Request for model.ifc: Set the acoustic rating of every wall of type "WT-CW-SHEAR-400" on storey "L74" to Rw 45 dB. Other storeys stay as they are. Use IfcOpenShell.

First a look at what the model holds.

```python
import ifcopenshell
import ifcopenshell.util.element

model = ifcopenshell.open("model.ifc")
print(model.schema)
storey = next(s for s in model.by_type("IfcBuildingStorey") if s.Name == "L74")
walls = [e for e in ifcopenshell.util.element.get_decomposition(storey) if e.is_a("IfcWall")]
seen = {}
for e in walls:
    element_type = ifcopenshell.util.element.get_type(e)
    key = (element_type.Name if element_type != e and element_type else None, ifcopenshell.util.element.get_pset(e, "Pset_WallCommon", "AcousticRating"))
    seen[key] = seen.get(key, 0) + 1
for (name, value), count in sorted(seen.items(), key=str):
    print(count, "x", name, "|", value)
```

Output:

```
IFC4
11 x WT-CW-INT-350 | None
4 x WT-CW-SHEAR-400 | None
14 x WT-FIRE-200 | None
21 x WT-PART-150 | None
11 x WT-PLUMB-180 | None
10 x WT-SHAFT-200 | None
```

```python
import ifcopenshell
import ifcopenshell.api.pset
import ifcopenshell.util.element

model = ifcopenshell.open("model.ifc")

storey = next(s for s in model.by_type("IfcBuildingStorey") if s.Name == "L74")
walls = [e for e in ifcopenshell.util.element.get_decomposition(storey) if e.is_a("IfcWall")]

count = 0
for e in walls:
    element_type = ifcopenshell.util.element.get_type(e)
    if element_type in (None, e) or element_type.Name != "WT-CW-SHEAR-400":
        continue
    found = ifcopenshell.util.element.get_pset(e, "Pset_WallCommon", should_inherit=False)
    if found:
        pset = model.by_id(found["id"])
        if len(ifcopenshell.util.element.get_elements_by_pset(pset)) > 1:
            pset = ifcopenshell.api.pset.unshare_pset(model, products=[e], pset=pset)[0]
    else:
        pset = ifcopenshell.api.pset.add_pset(model, product=e, name="Pset_WallCommon")
    ifcopenshell.api.pset.edit_pset(model, pset=pset, properties={"AcousticRating": "Rw 45 dB"})
    count += 1

print(count, "walls updated")

model.write("model-out.ifc")
```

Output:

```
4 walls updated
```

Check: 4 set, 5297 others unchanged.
